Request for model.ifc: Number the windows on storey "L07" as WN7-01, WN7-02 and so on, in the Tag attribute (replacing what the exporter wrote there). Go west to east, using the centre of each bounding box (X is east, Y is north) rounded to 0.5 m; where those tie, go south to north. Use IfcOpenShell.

First a look at what the model holds.

```python
import ifcopenshell
import ifcopenshell.util.element
import ifcopenshell.util.placement

model = ifcopenshell.open("model.ifc")
print(model.schema)
storey = next(s for s in model.by_type("IfcBuildingStorey") if s.Name == "L07")
windows = [e for e in ifcopenshell.util.element.get_decomposition(storey) if e.is_a("IfcWindow")]
for e in sorted(windows, key=lambda e: e.id()):
    origin = ifcopenshell.util.placement.get_local_placement(e.ObjectPlacement)[:3, 3]
    print(e.id(), e.Tag, e.Name, origin.round(2) + 0.0, sep=" | ")
```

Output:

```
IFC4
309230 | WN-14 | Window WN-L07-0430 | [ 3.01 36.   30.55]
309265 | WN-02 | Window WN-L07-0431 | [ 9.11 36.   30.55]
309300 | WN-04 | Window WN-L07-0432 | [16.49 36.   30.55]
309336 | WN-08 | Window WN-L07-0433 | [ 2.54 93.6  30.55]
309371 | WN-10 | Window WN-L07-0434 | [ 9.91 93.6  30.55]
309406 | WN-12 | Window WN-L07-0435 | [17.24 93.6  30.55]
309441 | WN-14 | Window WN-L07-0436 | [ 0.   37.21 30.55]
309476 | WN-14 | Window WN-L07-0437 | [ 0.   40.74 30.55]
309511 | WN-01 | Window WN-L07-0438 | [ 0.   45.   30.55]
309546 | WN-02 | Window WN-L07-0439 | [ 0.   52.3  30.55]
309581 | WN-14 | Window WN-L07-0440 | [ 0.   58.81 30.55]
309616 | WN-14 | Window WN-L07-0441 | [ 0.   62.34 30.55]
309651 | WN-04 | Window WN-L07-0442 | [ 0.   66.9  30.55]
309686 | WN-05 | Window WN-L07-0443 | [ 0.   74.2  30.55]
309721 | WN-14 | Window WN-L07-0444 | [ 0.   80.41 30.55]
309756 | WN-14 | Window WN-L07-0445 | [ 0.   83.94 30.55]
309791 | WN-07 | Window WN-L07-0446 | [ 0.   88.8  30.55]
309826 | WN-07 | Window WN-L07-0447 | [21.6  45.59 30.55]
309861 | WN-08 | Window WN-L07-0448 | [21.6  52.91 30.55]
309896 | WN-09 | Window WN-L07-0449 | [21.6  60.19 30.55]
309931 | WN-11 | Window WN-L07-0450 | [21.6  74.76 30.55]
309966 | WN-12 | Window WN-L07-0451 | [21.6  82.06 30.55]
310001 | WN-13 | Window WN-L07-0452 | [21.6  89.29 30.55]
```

```python
import ifcopenshell
import ifcopenshell.geom
import ifcopenshell.util.element
import ifcopenshell.util.shape

model = ifcopenshell.open("model.ifc")
settings = ifcopenshell.geom.settings()
settings.set("use-world-coords", True)


def centre(element):
    shape = ifcopenshell.geom.create_shape(settings, element)
    return ifcopenshell.util.shape.get_bbox_centroid(shape.geometry)


storey = next(s for s in model.by_type("IfcBuildingStorey") if s.Name == "L07")
windows = [e for e in ifcopenshell.util.element.get_decomposition(storey) if e.is_a("IfcWindow")]

# Insertion points can sit at a corner or the storey origin, so sort by the geometry (in metres).
centres = {e: centre(e) for e in windows}
windows.sort(key=lambda e: (round(centres[e][0] / 0.5), centres[e][1]))

for i, e in enumerate(windows, start=1):
    number = f"WN7-{i:02d}"
    e.Tag = number
    print(e.id(), number)

model.write("model-out.ifc")
```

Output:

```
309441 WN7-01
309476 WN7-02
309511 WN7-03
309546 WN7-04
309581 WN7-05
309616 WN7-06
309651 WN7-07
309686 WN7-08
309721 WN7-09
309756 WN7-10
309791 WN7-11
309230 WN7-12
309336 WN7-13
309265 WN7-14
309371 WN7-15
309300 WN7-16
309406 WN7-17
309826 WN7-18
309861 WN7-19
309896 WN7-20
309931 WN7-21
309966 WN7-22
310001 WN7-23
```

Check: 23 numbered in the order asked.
